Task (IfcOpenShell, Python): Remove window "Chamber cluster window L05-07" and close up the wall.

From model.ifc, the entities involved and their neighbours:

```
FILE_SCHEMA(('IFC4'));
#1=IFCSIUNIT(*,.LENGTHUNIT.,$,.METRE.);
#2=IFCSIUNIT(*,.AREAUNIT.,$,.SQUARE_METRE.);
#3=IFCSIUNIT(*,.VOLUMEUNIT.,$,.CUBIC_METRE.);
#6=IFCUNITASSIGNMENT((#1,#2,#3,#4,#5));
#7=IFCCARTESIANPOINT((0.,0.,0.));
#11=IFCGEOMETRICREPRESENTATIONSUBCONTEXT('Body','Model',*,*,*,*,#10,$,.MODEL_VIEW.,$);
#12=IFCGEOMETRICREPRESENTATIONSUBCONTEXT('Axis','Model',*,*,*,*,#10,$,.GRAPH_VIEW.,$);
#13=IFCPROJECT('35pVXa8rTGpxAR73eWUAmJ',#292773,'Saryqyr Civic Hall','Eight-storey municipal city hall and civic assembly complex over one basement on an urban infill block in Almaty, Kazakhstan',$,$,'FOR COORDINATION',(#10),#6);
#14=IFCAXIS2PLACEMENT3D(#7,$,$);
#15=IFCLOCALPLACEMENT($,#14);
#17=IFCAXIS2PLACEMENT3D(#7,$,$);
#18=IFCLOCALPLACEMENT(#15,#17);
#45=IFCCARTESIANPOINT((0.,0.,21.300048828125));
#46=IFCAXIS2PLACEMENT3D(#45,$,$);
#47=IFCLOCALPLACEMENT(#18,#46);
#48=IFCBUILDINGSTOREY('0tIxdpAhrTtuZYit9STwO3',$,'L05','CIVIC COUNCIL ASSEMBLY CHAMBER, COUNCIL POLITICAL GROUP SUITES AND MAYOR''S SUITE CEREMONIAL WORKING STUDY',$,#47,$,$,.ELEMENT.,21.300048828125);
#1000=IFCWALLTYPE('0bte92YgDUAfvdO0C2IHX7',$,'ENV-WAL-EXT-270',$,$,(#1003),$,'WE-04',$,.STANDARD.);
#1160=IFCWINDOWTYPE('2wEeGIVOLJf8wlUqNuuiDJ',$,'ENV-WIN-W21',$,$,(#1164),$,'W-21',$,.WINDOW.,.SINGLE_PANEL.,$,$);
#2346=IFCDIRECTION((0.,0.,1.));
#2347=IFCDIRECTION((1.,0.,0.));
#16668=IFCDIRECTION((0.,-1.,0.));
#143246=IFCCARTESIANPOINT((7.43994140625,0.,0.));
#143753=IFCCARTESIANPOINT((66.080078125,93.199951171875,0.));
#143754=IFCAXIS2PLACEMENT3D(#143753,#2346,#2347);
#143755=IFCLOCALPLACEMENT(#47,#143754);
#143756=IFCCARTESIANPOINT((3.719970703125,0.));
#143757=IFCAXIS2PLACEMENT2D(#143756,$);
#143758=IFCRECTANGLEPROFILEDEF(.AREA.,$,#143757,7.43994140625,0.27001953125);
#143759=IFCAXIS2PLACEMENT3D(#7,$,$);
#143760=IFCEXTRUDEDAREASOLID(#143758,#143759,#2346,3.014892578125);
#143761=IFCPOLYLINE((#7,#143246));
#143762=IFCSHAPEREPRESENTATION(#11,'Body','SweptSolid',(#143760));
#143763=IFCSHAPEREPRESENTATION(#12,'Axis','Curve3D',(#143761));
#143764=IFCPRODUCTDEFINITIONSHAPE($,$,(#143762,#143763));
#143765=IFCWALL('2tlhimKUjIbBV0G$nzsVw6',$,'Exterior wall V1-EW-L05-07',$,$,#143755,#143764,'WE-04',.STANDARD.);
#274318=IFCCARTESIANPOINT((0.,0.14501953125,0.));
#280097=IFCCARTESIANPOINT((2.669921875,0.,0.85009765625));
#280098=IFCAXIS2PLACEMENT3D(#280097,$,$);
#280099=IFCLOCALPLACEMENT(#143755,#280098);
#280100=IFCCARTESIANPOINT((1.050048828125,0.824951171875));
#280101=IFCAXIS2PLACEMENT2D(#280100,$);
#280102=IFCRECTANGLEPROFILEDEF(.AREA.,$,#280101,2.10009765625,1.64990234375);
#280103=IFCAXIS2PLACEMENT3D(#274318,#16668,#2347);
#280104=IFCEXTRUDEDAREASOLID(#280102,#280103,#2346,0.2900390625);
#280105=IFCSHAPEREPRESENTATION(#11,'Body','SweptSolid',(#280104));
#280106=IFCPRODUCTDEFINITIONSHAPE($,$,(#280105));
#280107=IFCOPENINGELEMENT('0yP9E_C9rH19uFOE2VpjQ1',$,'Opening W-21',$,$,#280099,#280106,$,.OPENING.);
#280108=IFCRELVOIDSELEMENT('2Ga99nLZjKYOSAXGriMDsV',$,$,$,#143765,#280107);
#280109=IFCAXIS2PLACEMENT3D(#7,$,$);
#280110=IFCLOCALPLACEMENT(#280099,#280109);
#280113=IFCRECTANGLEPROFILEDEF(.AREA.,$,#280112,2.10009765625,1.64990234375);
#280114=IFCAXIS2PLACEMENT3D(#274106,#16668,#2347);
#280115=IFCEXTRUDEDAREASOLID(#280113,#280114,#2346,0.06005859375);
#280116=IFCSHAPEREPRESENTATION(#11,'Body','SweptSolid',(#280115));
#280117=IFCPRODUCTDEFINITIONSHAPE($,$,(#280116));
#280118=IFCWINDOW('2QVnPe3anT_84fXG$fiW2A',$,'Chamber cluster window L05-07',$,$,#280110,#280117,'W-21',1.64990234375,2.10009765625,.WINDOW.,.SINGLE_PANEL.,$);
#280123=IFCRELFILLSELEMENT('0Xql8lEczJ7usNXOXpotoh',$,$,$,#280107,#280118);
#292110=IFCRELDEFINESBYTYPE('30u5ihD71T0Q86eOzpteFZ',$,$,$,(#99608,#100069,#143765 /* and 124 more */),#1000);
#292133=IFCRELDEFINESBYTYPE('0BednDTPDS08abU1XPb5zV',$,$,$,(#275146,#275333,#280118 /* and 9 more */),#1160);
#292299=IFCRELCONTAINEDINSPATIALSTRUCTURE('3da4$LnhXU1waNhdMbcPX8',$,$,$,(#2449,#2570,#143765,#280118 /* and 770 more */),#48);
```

```python
import ifcopenshell
import ifcopenshell.api.feature
import ifcopenshell.api.root
import ifcopenshell.geom
import ifcopenshell.util.shape

model = ifcopenshell.open("model.ifc")
settings = ifcopenshell.geom.settings()


def volume(element):
    """Net volume in cubic metres, openings subtracted."""
    shape = ifcopenshell.geom.create_shape(settings, element)
    return ifcopenshell.util.shape.get_volume(shape.geometry)


window = model.by_id(280118)
opening = window.FillsVoids[0].RelatingOpeningElement
wall = opening.VoidsElements[0].RelatingBuildingElement
before = volume(wall)

ifcopenshell.api.root.remove_product(model, product=window)
ifcopenshell.api.feature.remove_feature(model, feature=opening)

after = volume(wall)

print(f"wall volume {before:.3f} -> {after:.3f} m3")

model.write("model_v2.ifc")
```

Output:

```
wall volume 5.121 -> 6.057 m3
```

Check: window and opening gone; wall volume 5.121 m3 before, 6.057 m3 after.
